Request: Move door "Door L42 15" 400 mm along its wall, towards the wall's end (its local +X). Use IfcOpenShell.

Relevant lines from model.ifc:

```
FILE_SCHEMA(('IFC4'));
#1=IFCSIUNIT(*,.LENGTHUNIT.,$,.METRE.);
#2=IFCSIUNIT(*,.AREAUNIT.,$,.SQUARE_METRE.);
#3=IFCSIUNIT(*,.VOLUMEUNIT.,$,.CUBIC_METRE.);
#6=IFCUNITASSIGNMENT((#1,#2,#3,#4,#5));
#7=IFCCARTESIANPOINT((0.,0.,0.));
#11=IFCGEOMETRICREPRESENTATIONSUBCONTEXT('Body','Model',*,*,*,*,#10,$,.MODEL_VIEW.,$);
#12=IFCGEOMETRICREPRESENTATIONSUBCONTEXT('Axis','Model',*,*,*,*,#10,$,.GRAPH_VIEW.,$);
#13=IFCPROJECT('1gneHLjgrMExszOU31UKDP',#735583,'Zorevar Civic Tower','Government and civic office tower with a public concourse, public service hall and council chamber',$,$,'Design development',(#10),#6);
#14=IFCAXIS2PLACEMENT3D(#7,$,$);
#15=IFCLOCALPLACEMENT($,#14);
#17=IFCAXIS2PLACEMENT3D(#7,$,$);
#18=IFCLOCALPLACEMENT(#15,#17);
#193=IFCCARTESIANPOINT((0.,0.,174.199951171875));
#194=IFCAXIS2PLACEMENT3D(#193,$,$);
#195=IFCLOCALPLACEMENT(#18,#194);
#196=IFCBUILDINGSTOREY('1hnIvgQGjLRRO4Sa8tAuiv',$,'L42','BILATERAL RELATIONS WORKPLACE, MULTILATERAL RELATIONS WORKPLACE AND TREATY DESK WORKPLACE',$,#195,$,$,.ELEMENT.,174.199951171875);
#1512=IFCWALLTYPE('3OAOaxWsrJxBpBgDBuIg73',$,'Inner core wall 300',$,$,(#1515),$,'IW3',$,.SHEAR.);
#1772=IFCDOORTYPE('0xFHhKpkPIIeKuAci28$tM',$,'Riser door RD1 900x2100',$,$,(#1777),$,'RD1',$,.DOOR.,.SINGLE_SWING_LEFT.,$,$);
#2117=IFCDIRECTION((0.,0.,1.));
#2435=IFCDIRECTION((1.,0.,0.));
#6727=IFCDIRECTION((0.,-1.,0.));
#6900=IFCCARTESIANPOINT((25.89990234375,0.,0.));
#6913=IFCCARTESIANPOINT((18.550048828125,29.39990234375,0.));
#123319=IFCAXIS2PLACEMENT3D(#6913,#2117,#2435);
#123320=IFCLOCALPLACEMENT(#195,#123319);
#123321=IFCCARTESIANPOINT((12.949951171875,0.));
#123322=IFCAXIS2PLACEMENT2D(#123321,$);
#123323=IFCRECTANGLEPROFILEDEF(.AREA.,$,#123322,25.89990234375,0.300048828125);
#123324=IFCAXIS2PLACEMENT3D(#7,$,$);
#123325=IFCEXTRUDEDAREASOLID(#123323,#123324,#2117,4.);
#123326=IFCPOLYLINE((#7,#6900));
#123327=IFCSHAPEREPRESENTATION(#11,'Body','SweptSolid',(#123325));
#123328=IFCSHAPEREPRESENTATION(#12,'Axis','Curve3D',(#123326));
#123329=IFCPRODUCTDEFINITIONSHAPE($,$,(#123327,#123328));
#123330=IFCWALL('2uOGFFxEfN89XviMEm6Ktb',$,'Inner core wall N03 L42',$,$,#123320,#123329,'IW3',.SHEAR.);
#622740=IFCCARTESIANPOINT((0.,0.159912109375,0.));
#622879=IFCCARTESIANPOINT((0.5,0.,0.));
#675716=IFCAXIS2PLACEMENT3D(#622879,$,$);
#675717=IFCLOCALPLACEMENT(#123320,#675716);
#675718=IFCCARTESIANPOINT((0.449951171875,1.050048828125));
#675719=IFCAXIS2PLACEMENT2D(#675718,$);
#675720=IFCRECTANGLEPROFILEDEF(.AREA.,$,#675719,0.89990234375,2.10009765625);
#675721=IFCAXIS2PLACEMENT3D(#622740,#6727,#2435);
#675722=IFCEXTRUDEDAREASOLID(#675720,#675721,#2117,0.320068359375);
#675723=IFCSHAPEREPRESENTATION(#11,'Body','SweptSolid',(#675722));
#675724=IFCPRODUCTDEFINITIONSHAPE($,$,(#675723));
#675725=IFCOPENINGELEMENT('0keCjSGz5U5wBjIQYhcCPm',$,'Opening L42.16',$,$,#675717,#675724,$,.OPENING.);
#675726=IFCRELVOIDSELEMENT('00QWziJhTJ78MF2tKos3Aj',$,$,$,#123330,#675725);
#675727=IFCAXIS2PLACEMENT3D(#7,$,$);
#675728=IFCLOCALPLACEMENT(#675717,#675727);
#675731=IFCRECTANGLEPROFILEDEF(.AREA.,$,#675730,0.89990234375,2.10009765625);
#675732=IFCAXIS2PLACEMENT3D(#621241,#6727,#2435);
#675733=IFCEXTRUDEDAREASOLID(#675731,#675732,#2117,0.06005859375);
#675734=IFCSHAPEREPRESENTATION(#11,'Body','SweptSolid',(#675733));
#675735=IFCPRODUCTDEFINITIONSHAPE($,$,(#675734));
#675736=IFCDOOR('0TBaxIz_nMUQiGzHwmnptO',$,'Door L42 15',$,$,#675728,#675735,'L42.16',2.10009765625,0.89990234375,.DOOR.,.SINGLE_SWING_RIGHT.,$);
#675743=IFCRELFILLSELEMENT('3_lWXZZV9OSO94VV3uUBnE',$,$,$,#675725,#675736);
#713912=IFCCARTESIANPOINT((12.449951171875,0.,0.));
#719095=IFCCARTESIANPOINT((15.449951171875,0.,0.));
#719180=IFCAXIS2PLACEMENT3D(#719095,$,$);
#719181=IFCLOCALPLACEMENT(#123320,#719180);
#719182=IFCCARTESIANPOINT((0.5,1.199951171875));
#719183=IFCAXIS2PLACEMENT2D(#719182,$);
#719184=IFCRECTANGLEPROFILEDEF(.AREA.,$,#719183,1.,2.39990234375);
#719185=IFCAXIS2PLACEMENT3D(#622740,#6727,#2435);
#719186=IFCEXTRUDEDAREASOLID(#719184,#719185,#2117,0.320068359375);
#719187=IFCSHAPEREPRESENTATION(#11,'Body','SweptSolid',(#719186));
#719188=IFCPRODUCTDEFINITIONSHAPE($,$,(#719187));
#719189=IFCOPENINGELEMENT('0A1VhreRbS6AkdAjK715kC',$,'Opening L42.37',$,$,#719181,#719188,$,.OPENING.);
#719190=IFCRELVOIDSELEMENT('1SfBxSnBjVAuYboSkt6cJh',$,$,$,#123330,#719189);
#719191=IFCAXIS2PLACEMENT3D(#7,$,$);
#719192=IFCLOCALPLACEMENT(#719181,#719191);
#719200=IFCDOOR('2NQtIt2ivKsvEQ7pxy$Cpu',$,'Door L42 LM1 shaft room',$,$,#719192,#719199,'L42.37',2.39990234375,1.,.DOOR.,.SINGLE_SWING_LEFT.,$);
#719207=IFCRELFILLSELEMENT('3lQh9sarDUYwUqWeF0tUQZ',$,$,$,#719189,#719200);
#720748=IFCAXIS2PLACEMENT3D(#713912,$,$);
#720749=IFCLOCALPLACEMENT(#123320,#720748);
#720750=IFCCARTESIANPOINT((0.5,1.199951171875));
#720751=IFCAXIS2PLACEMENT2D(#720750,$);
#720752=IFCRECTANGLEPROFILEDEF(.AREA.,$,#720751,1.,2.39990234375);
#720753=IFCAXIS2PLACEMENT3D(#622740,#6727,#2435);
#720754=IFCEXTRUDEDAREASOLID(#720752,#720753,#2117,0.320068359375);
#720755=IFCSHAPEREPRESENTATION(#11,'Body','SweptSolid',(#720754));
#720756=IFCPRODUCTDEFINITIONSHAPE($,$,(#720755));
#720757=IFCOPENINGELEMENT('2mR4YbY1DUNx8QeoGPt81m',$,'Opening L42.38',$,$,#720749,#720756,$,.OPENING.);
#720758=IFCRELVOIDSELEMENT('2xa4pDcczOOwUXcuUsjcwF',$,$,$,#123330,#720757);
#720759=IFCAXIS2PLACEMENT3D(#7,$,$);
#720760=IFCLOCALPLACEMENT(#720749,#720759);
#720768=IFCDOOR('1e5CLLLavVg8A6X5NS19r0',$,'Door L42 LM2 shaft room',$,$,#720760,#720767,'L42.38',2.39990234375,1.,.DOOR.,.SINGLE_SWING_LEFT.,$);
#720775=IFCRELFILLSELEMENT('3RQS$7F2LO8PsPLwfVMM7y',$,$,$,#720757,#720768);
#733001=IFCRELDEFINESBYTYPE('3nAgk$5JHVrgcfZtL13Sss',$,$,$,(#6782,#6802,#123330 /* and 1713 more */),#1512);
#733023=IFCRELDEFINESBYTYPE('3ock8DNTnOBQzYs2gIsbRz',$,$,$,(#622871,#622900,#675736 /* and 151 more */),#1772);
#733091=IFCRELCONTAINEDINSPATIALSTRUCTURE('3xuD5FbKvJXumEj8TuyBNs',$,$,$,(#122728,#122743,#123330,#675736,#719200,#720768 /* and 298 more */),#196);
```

```python
import ifcopenshell
import ifcopenshell.api.geometry
import ifcopenshell.util.placement

model = ifcopenshell.open("model.ifc")

door = model.by_guid("0TBaxIz_nMUQiGzHwmnptO")
opening = door.FillsVoids[0].RelatingOpeningElement
wall = opening.VoidsElements[0].RelatingBuildingElement

wall_matrix = ifcopenshell.util.placement.get_local_placement(wall.ObjectPlacement)
shift = wall_matrix[:3, 0] * 0.4
before = ifcopenshell.util.placement.get_local_placement(door.ObjectPlacement)[:3, 3].copy()

# The door is placed relative to its opening, so it follows when the opening moves.
matrix = ifcopenshell.util.placement.get_local_placement(opening.ObjectPlacement)
matrix[:3, 3] += shift
ifcopenshell.api.geometry.edit_object_placement(
    model, product=opening, matrix=matrix, is_si=False, should_transform_children=True
)

after = ifcopenshell.util.placement.get_local_placement(door.ObjectPlacement)[:3, 3]
print("door moved by", (after - before).round(3) + 0.0)

model.write("model_updated.ifc")
```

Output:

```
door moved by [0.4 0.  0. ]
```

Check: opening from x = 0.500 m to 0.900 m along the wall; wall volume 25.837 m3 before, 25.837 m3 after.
